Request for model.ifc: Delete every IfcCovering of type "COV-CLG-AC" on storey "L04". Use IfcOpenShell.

First a look at what the model holds.

```python
import ifcopenshell
import ifcopenshell.util.element

model = ifcopenshell.open("model.ifc")
print(model.schema)
storey = next(s for s in model.by_type("IfcBuildingStorey") if s.Name == "L04")
coverings = [e for e in ifcopenshell.util.element.get_decomposition(storey) if e.is_a("IfcCovering")]
seen = {}
for e in coverings:
    element_type = ifcopenshell.util.element.get_type(e)
    name = element_type.Name if element_type not in (None, e) else None
    seen[name] = seen.get(name, 0) + 1
for name, count in sorted(seen.items(), key=str):
    print(count, "x", name)
```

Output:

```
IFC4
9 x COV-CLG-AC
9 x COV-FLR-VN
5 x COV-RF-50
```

```python
import ifcopenshell
import ifcopenshell.api.root
import ifcopenshell.util.element

model = ifcopenshell.open("model.ifc")

storey = next(s for s in model.by_type("IfcBuildingStorey") if s.Name == "L04")
coverings = [e for e in ifcopenshell.util.element.get_decomposition(storey) if e.is_a("IfcCovering")]
targets = [e for e in coverings if (t := ifcopenshell.util.element.get_type(e)) not in (None, e) and t.Name == "COV-CLG-AC"]

for e in targets:
    ifcopenshell.api.root.remove_product(model, product=e)
print(len(targets), "removed")

model.write("model_updated.ifc")
```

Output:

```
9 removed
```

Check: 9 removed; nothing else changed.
